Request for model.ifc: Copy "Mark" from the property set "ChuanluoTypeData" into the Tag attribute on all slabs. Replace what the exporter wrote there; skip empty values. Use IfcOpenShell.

First a look at what the model holds.

```python
import ifcopenshell
import ifcopenshell.util.element

model = ifcopenshell.open("model.ifc")
print(model.schema)
slabs = model.by_type("IfcSlab")
print(len(slabs), "slabs")
for e in slabs[:8]:
    source = ifcopenshell.util.element.get_pset(e, "ChuanluoTypeData", "Mark")
    target = e.Tag
    print(e.id(), repr(source), repr(target), sep=" | ")
```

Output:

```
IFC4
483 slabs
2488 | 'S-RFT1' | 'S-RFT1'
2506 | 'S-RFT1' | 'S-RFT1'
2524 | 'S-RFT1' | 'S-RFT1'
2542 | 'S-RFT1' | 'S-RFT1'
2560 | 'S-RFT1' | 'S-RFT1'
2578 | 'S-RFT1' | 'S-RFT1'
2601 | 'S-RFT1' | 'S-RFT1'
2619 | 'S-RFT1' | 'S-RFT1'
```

```python
import ifcopenshell
import ifcopenshell.util.element

model = ifcopenshell.open("model.ifc")

count = 0
for e in model.by_type("IfcSlab"):
    value = ifcopenshell.util.element.get_pset(e, "ChuanluoTypeData", "Mark")
    current = e.Tag
    if not value or not value.strip() or current == value:
        continue
    e.Tag = value
    count += 1

print(count, "slabs updated")

model.write("model_rev.ifc")
```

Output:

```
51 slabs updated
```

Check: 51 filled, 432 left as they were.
